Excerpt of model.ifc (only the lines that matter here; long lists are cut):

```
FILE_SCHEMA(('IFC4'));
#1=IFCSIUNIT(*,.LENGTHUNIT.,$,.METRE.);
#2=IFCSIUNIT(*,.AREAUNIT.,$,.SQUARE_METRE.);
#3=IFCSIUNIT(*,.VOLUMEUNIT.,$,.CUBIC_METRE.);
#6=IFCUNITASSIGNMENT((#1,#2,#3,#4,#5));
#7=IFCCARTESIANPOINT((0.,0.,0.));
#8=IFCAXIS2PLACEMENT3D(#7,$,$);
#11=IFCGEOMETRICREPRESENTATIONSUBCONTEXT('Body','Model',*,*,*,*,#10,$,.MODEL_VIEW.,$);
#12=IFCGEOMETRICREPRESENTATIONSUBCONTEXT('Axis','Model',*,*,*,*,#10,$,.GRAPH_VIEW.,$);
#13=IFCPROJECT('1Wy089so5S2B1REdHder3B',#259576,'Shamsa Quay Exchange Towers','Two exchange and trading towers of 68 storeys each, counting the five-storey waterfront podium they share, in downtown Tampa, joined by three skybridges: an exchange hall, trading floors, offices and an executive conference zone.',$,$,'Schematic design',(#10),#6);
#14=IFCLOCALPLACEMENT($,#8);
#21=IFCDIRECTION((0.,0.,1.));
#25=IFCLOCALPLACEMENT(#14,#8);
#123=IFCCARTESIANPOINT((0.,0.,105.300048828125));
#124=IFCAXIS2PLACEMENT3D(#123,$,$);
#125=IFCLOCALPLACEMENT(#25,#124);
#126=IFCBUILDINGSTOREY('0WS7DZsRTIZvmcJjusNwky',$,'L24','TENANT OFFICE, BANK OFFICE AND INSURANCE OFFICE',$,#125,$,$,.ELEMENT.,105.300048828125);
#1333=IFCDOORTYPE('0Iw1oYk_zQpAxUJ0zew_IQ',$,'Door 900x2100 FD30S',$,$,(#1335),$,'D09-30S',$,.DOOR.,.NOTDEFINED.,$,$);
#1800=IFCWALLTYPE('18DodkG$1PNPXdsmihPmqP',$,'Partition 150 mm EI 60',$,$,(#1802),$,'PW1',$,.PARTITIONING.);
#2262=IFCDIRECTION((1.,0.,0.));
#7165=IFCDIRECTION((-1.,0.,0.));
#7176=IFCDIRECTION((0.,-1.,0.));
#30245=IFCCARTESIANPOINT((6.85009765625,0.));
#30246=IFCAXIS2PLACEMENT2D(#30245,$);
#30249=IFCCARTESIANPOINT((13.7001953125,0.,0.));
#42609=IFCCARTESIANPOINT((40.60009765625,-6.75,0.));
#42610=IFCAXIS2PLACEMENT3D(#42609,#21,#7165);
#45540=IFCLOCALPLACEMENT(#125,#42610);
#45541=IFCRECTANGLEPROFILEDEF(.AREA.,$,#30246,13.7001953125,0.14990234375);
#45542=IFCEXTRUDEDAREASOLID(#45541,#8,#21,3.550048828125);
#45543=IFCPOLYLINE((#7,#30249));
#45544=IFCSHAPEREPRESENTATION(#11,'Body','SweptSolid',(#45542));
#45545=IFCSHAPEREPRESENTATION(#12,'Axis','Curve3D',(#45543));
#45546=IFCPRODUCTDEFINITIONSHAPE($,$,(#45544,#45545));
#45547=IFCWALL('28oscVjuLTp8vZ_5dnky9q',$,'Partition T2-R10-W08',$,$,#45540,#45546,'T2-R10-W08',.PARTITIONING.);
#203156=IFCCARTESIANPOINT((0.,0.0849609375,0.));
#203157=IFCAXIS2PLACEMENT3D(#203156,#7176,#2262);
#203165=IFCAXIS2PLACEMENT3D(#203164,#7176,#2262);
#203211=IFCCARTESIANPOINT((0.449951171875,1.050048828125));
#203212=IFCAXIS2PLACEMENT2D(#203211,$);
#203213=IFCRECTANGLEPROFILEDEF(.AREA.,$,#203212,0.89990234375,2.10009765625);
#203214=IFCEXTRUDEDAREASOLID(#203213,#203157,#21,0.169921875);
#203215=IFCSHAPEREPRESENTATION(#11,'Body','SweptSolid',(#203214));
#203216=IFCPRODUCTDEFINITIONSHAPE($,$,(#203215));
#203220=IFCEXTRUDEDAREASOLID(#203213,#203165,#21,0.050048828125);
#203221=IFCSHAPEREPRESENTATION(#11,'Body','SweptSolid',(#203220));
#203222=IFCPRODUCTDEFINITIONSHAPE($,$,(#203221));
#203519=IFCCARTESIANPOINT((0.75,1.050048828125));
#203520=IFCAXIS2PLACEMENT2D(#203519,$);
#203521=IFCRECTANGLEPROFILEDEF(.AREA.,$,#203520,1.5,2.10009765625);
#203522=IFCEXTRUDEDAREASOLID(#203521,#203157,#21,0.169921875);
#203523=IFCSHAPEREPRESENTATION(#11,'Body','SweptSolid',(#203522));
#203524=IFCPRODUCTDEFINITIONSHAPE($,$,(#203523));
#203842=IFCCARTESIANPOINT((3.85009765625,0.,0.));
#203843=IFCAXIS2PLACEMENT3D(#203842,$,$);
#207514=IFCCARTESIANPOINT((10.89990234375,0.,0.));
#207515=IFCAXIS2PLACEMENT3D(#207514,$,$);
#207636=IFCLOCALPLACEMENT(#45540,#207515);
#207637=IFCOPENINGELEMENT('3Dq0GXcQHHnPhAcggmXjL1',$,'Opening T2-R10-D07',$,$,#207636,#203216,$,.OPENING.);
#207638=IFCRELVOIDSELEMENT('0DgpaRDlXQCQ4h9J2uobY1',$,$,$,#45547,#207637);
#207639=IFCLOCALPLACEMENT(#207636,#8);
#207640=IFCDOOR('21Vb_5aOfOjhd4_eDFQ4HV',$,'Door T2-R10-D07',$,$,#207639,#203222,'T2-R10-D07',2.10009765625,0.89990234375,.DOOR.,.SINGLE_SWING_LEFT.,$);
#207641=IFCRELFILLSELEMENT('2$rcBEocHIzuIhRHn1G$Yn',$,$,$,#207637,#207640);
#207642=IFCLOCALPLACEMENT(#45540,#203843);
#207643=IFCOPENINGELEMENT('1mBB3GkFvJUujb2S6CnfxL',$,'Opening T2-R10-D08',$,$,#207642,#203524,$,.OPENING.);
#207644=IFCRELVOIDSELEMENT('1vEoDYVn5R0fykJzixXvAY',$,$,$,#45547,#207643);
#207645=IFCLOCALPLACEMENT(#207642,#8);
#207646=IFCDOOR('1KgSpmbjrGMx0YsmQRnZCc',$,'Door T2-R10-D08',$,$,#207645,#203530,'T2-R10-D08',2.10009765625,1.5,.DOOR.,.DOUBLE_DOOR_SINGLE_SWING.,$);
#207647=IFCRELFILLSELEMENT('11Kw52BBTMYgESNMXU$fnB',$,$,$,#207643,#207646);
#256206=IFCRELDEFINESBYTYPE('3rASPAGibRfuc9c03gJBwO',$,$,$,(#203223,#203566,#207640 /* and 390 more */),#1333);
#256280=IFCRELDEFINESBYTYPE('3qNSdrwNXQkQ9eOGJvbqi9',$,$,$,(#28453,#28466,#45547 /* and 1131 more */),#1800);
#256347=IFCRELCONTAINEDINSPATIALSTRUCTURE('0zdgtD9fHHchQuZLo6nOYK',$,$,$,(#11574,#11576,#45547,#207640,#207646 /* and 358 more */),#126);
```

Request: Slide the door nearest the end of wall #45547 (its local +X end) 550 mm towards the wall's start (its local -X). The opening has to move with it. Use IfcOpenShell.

```python
import ifcopenshell
import ifcopenshell.api.geometry
import ifcopenshell.util.placement

model = ifcopenshell.open("model.ifc")

door = model.by_guid("21Vb_5aOfOjhd4_eDFQ4HV")
opening = door.FillsVoids[0].RelatingOpeningElement
wall = opening.VoidsElements[0].RelatingBuildingElement

wall_matrix = ifcopenshell.util.placement.get_local_placement(wall.ObjectPlacement)
shift = wall_matrix[:3, 0] * -0.55
before = ifcopenshell.util.placement.get_local_placement(door.ObjectPlacement)[:3, 3].copy()

# The door is placed relative to its opening, so it follows when the opening moves.
matrix = ifcopenshell.util.placement.get_local_placement(opening.ObjectPlacement)
matrix[:3, 3] += shift
ifcopenshell.api.geometry.edit_object_placement(
    model, product=opening, matrix=matrix, is_si=False, should_transform_children=True
)

after = ifcopenshell.util.placement.get_local_placement(door.ObjectPlacement)[:3, 3]
print("door moved by", (after - before).round(3) + 0.0)

model.write("model_updated.ifc")
```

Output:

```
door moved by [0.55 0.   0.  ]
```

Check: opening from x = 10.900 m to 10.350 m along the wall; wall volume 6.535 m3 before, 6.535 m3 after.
